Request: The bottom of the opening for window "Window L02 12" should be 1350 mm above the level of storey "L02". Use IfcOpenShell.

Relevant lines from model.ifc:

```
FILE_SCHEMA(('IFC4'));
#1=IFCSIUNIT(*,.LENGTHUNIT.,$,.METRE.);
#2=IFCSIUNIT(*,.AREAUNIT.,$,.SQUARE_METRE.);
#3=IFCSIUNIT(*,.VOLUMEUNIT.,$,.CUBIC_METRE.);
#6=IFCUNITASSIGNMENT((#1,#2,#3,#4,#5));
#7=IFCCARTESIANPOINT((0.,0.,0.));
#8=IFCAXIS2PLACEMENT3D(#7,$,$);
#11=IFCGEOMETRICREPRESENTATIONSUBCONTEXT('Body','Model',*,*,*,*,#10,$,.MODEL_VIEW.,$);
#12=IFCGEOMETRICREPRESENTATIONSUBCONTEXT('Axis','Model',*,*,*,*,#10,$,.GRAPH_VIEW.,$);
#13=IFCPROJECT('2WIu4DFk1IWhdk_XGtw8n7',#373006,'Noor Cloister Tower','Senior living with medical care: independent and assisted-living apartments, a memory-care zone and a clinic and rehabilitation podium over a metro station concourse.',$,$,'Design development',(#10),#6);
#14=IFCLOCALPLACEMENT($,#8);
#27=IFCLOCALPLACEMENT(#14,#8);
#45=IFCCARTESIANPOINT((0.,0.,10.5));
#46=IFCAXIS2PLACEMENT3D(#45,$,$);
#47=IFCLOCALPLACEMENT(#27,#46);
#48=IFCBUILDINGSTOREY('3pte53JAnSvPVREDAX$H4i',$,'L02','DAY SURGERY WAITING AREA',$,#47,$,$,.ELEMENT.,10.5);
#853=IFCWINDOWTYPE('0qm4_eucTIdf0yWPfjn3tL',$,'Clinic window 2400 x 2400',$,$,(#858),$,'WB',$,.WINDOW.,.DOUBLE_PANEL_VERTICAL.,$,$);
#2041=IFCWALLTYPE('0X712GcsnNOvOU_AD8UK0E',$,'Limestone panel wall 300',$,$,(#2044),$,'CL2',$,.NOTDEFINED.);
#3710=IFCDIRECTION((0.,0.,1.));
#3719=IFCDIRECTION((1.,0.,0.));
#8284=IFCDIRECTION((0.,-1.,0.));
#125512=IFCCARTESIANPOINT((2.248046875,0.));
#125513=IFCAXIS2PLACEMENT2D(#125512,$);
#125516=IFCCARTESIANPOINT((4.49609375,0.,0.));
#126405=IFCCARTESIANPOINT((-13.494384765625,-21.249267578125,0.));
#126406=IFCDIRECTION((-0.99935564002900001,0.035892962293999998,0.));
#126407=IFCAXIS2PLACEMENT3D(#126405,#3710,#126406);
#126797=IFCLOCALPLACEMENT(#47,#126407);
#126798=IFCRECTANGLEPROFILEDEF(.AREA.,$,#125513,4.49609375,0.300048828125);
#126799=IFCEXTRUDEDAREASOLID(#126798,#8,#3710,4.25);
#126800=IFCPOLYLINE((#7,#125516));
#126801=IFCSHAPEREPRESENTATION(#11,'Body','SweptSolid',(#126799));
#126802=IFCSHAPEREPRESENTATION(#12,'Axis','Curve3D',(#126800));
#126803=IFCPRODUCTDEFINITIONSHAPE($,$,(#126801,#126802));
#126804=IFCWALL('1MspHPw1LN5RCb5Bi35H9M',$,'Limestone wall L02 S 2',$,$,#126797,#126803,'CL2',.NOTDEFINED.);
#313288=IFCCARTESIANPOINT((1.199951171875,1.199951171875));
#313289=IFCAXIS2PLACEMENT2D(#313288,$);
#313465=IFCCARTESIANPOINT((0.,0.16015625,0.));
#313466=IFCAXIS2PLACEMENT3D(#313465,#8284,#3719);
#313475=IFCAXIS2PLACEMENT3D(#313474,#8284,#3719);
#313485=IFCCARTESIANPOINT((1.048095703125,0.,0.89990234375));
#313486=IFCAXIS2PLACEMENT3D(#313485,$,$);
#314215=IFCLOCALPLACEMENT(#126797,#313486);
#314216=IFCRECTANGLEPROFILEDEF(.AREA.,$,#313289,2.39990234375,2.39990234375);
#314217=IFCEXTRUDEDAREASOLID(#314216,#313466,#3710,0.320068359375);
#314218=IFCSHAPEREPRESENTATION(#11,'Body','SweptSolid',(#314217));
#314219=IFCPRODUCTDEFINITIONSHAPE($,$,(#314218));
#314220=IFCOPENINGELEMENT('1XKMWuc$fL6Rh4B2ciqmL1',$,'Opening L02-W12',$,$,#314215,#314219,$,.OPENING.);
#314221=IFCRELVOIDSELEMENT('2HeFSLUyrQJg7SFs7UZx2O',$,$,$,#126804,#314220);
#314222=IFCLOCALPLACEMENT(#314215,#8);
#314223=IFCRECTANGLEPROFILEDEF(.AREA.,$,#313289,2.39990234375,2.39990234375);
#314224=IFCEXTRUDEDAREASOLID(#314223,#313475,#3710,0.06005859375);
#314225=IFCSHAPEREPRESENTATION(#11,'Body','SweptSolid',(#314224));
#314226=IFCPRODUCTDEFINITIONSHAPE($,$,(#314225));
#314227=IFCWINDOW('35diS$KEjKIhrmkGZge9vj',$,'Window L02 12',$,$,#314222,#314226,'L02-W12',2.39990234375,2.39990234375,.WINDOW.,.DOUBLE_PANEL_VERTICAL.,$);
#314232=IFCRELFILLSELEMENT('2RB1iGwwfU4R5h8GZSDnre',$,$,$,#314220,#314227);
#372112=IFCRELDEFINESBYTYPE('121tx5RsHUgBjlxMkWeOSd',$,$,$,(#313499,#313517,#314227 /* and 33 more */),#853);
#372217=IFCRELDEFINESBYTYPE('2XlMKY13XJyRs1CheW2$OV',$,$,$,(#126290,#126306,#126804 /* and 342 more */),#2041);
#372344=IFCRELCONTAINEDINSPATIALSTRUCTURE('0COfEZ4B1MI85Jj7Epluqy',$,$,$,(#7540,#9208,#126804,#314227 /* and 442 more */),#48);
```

```python
import numpy as np
import ifcopenshell
import ifcopenshell.api.geometry
import ifcopenshell.geom
import ifcopenshell.util.element
import ifcopenshell.util.placement
import ifcopenshell.util.shape
import ifcopenshell.util.unit

model = ifcopenshell.open("model.ifc")
unit_scale = ifcopenshell.util.unit.calculate_unit_scale(model)

window = model.by_guid("35diS$KEjKIhrmkGZge9vj")
opening = window.FillsVoids[0].RelatingOpeningElement
storey = ifcopenshell.util.element.get_container(window, ifc_class="IfcBuildingStorey")
level = ifcopenshell.util.placement.get_local_placement(storey.ObjectPlacement)[2, 3]

# The opening's origin need not be at the sill, so measure its lowest point.
shape = ifcopenshell.geom.create_shape(ifcopenshell.geom.settings(), opening)
bottom = ifcopenshell.util.shape.get_shape_bottom_elevation(shape, shape.geometry) / unit_scale
dz = level + 1.35 - bottom

shift = np.array([0.0, 0.0, dz])
# The window is placed relative to its opening, so it follows when the opening moves.
matrix = ifcopenshell.util.placement.get_local_placement(opening.ObjectPlacement)
matrix[:3, 3] += shift
ifcopenshell.api.geometry.edit_object_placement(
    model, product=opening, matrix=matrix, is_si=False, should_transform_children=True
)

print(f"moved by {dz * unit_scale:+.3f} m")

model.write("model_rev.ifc")
```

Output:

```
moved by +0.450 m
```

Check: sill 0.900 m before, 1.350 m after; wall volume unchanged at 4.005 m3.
